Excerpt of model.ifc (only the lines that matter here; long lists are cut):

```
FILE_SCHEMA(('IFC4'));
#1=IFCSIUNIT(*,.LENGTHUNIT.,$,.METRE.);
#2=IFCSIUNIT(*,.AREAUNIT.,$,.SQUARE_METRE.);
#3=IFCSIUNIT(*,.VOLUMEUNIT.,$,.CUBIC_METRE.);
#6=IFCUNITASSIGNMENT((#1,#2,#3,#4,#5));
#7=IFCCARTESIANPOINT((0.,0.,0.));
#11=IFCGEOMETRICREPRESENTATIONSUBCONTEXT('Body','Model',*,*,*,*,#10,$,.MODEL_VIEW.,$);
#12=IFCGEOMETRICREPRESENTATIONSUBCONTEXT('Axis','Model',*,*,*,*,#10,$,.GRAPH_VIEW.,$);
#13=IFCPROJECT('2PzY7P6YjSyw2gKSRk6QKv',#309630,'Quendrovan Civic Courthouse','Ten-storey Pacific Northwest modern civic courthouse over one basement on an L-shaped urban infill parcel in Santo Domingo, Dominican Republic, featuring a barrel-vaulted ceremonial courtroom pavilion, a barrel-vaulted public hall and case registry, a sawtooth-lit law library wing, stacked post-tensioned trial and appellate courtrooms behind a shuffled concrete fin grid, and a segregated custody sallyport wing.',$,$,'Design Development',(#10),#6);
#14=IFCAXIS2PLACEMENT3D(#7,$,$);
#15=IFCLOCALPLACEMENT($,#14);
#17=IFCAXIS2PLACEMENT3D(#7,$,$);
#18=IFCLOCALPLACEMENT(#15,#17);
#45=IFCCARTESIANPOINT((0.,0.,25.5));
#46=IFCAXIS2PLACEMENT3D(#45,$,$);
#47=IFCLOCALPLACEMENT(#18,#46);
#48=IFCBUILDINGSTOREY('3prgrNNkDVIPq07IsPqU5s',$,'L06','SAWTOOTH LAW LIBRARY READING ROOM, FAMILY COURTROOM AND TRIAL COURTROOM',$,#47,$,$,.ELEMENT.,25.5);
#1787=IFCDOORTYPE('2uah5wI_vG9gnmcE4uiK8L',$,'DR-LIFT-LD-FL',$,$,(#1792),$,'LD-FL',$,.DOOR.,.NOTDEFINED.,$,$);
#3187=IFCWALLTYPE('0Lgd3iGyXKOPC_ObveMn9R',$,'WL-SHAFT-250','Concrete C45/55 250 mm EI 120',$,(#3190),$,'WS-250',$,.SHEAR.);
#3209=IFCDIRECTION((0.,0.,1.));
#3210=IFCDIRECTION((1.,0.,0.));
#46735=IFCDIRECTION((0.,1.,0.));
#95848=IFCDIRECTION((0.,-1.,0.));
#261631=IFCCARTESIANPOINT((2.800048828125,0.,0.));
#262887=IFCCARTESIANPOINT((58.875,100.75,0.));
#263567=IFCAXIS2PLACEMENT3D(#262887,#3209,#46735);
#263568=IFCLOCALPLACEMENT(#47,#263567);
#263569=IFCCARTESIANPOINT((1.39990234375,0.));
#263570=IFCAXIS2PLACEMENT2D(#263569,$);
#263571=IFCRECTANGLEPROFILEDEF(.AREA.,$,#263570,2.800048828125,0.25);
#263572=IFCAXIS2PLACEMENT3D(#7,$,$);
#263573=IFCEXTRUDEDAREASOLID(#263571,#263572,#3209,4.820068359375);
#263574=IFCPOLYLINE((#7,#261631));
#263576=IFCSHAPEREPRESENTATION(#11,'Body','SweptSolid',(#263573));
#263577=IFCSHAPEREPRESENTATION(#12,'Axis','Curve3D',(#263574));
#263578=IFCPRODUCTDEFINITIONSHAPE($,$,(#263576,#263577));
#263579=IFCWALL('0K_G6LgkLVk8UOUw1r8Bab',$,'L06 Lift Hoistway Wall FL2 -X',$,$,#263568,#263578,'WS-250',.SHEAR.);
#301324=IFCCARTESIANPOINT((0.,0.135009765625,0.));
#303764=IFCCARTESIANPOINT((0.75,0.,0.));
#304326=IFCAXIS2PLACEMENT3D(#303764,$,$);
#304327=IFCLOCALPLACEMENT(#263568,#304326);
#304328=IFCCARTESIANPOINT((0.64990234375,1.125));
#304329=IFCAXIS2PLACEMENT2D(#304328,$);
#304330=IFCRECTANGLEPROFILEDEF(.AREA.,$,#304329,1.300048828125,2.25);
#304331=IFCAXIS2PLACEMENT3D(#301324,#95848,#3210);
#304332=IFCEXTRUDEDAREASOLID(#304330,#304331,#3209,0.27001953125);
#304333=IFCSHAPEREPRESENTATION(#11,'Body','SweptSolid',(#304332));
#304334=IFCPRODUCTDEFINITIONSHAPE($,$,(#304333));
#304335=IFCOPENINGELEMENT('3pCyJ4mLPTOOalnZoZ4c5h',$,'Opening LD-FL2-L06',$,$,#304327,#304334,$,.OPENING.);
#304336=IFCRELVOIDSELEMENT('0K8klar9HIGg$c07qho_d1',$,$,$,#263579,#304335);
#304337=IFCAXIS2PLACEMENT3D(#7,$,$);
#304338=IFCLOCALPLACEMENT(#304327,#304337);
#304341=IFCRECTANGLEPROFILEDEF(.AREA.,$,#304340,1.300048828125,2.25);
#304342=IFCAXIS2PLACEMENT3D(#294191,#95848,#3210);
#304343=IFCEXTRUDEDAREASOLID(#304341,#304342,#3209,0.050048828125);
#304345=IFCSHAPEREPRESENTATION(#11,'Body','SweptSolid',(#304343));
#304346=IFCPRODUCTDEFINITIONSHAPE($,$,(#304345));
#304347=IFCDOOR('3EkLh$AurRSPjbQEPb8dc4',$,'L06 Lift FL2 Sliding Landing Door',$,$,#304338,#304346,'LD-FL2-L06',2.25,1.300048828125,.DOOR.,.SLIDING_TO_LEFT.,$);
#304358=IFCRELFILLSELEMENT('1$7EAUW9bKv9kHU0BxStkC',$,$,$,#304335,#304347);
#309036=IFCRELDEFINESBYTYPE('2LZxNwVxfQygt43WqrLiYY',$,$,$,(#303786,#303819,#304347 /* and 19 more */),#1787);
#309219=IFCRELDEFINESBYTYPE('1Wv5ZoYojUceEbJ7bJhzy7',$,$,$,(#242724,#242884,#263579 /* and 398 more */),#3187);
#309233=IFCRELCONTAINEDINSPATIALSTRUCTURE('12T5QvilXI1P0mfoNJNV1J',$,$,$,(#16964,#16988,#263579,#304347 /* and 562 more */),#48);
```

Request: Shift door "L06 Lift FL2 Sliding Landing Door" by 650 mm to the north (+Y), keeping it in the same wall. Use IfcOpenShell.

```python
import ifcopenshell
import ifcopenshell.api.geometry
import ifcopenshell.util.placement

model = ifcopenshell.open("model.ifc")

door = model.by_guid("3EkLh$AurRSPjbQEPb8dc4")
opening = door.FillsVoids[0].RelatingOpeningElement
wall = opening.VoidsElements[0].RelatingBuildingElement

wall_matrix = ifcopenshell.util.placement.get_local_placement(wall.ObjectPlacement)
shift = wall_matrix[:3, 0] * 0.65
before = ifcopenshell.util.placement.get_local_placement(door.ObjectPlacement)[:3, 3].copy()

# The door is placed relative to its opening, so it follows when the opening moves.
matrix = ifcopenshell.util.placement.get_local_placement(opening.ObjectPlacement)
matrix[:3, 3] += shift
ifcopenshell.api.geometry.edit_object_placement(
    model, product=opening, matrix=matrix, is_si=False, should_transform_children=True
)

after = ifcopenshell.util.placement.get_local_placement(door.ObjectPlacement)[:3, 3]
print("door moved by", (after - before).round(3) + 0.0)

model.write("model_edited.ifc")
```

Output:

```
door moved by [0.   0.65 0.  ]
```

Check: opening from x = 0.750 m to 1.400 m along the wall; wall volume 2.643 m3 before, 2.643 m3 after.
